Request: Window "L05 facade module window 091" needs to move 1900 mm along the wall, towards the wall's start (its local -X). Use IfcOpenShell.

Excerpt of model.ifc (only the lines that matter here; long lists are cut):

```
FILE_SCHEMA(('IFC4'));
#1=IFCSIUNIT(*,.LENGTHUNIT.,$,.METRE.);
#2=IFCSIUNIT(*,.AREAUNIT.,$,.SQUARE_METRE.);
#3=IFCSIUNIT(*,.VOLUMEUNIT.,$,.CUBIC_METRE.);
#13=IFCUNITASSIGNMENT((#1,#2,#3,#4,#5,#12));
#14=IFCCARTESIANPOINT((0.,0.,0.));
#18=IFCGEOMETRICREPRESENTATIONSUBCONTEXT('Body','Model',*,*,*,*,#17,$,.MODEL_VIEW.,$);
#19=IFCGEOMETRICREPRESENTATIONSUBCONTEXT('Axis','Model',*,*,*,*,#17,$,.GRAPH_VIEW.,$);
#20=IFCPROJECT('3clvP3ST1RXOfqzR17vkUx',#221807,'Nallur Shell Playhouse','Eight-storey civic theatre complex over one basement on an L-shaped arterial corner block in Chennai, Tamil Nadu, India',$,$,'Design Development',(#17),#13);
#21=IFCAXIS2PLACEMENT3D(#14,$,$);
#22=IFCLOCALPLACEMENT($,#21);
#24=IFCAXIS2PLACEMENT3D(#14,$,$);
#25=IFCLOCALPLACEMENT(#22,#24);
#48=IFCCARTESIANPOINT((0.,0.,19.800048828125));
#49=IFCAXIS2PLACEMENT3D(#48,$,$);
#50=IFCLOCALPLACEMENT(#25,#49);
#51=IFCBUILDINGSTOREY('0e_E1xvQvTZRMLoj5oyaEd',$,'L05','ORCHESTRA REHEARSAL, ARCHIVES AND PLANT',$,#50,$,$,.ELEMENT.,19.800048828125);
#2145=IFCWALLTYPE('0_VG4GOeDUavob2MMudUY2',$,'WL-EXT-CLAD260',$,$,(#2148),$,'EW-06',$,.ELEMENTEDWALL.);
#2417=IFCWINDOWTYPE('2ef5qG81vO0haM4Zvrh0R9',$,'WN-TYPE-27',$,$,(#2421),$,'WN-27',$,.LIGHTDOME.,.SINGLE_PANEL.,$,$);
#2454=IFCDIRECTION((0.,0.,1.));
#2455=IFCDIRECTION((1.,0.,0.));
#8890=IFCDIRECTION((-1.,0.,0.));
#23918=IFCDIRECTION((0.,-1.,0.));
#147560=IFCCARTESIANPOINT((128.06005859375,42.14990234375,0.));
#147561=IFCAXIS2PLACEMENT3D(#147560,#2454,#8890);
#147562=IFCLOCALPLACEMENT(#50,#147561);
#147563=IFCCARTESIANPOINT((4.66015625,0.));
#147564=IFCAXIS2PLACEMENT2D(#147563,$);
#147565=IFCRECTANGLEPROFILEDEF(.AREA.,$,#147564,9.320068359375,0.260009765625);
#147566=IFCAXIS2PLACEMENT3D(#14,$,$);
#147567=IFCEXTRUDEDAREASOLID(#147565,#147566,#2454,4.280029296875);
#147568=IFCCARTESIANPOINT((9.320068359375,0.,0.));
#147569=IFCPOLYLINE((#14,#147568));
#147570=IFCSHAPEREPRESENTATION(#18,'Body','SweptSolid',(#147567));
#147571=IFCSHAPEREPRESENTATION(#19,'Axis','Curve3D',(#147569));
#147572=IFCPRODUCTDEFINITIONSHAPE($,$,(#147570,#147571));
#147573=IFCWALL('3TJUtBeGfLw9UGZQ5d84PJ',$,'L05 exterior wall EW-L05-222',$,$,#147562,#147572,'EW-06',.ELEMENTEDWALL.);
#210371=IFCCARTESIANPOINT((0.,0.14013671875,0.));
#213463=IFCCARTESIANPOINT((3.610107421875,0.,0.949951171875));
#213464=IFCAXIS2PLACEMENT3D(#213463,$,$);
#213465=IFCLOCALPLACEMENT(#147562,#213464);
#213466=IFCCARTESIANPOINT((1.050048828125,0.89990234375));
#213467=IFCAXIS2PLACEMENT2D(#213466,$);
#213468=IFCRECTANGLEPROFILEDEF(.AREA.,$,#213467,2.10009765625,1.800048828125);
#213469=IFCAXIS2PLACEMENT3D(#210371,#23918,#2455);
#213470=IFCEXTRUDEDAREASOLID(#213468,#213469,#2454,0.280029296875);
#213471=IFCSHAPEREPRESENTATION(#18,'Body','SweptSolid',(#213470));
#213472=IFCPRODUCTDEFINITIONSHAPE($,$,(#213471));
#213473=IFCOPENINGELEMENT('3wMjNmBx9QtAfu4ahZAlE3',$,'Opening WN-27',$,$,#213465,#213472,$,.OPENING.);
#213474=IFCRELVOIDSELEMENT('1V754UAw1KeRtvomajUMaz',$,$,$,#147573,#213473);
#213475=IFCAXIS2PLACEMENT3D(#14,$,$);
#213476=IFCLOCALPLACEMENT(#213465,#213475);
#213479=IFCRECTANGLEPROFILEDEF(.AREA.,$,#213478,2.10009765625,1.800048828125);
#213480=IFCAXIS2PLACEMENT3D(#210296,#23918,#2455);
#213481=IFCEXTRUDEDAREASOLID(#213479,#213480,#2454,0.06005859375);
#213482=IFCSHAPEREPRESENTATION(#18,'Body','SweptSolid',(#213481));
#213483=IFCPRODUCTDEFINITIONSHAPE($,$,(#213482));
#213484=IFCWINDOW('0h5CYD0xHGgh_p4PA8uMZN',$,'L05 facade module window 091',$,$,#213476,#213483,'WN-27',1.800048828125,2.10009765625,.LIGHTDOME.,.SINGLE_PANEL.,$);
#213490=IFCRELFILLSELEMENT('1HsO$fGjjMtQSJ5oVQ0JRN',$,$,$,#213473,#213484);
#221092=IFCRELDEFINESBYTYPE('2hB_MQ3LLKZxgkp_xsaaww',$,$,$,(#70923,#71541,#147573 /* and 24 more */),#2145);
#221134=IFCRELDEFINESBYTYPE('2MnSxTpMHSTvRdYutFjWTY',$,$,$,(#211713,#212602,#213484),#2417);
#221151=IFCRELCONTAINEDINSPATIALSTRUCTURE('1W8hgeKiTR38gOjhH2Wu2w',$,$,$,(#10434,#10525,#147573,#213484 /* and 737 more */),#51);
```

```python
import ifcopenshell
import ifcopenshell.api.geometry
import ifcopenshell.util.placement

model = ifcopenshell.open("model.ifc")

window = model.by_id(213484)
opening = window.FillsVoids[0].RelatingOpeningElement
wall = opening.VoidsElements[0].RelatingBuildingElement

wall_matrix = ifcopenshell.util.placement.get_local_placement(wall.ObjectPlacement)
shift = wall_matrix[:3, 0] * -1.9
before = ifcopenshell.util.placement.get_local_placement(window.ObjectPlacement)[:3, 3].copy()

# The window is placed relative to its opening, so it follows when the opening moves.
matrix = ifcopenshell.util.placement.get_local_placement(opening.ObjectPlacement)
matrix[:3, 3] += shift
ifcopenshell.api.geometry.edit_object_placement(
    model, product=opening, matrix=matrix, is_si=False, should_transform_children=True
)

after = ifcopenshell.util.placement.get_local_placement(window.ObjectPlacement)[:3, 3]
print("window moved by", (after - before).round(3) + 0.0)

model.write("model-out.ifc")
```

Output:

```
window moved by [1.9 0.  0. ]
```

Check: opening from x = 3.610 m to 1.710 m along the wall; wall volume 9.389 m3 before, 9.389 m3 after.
